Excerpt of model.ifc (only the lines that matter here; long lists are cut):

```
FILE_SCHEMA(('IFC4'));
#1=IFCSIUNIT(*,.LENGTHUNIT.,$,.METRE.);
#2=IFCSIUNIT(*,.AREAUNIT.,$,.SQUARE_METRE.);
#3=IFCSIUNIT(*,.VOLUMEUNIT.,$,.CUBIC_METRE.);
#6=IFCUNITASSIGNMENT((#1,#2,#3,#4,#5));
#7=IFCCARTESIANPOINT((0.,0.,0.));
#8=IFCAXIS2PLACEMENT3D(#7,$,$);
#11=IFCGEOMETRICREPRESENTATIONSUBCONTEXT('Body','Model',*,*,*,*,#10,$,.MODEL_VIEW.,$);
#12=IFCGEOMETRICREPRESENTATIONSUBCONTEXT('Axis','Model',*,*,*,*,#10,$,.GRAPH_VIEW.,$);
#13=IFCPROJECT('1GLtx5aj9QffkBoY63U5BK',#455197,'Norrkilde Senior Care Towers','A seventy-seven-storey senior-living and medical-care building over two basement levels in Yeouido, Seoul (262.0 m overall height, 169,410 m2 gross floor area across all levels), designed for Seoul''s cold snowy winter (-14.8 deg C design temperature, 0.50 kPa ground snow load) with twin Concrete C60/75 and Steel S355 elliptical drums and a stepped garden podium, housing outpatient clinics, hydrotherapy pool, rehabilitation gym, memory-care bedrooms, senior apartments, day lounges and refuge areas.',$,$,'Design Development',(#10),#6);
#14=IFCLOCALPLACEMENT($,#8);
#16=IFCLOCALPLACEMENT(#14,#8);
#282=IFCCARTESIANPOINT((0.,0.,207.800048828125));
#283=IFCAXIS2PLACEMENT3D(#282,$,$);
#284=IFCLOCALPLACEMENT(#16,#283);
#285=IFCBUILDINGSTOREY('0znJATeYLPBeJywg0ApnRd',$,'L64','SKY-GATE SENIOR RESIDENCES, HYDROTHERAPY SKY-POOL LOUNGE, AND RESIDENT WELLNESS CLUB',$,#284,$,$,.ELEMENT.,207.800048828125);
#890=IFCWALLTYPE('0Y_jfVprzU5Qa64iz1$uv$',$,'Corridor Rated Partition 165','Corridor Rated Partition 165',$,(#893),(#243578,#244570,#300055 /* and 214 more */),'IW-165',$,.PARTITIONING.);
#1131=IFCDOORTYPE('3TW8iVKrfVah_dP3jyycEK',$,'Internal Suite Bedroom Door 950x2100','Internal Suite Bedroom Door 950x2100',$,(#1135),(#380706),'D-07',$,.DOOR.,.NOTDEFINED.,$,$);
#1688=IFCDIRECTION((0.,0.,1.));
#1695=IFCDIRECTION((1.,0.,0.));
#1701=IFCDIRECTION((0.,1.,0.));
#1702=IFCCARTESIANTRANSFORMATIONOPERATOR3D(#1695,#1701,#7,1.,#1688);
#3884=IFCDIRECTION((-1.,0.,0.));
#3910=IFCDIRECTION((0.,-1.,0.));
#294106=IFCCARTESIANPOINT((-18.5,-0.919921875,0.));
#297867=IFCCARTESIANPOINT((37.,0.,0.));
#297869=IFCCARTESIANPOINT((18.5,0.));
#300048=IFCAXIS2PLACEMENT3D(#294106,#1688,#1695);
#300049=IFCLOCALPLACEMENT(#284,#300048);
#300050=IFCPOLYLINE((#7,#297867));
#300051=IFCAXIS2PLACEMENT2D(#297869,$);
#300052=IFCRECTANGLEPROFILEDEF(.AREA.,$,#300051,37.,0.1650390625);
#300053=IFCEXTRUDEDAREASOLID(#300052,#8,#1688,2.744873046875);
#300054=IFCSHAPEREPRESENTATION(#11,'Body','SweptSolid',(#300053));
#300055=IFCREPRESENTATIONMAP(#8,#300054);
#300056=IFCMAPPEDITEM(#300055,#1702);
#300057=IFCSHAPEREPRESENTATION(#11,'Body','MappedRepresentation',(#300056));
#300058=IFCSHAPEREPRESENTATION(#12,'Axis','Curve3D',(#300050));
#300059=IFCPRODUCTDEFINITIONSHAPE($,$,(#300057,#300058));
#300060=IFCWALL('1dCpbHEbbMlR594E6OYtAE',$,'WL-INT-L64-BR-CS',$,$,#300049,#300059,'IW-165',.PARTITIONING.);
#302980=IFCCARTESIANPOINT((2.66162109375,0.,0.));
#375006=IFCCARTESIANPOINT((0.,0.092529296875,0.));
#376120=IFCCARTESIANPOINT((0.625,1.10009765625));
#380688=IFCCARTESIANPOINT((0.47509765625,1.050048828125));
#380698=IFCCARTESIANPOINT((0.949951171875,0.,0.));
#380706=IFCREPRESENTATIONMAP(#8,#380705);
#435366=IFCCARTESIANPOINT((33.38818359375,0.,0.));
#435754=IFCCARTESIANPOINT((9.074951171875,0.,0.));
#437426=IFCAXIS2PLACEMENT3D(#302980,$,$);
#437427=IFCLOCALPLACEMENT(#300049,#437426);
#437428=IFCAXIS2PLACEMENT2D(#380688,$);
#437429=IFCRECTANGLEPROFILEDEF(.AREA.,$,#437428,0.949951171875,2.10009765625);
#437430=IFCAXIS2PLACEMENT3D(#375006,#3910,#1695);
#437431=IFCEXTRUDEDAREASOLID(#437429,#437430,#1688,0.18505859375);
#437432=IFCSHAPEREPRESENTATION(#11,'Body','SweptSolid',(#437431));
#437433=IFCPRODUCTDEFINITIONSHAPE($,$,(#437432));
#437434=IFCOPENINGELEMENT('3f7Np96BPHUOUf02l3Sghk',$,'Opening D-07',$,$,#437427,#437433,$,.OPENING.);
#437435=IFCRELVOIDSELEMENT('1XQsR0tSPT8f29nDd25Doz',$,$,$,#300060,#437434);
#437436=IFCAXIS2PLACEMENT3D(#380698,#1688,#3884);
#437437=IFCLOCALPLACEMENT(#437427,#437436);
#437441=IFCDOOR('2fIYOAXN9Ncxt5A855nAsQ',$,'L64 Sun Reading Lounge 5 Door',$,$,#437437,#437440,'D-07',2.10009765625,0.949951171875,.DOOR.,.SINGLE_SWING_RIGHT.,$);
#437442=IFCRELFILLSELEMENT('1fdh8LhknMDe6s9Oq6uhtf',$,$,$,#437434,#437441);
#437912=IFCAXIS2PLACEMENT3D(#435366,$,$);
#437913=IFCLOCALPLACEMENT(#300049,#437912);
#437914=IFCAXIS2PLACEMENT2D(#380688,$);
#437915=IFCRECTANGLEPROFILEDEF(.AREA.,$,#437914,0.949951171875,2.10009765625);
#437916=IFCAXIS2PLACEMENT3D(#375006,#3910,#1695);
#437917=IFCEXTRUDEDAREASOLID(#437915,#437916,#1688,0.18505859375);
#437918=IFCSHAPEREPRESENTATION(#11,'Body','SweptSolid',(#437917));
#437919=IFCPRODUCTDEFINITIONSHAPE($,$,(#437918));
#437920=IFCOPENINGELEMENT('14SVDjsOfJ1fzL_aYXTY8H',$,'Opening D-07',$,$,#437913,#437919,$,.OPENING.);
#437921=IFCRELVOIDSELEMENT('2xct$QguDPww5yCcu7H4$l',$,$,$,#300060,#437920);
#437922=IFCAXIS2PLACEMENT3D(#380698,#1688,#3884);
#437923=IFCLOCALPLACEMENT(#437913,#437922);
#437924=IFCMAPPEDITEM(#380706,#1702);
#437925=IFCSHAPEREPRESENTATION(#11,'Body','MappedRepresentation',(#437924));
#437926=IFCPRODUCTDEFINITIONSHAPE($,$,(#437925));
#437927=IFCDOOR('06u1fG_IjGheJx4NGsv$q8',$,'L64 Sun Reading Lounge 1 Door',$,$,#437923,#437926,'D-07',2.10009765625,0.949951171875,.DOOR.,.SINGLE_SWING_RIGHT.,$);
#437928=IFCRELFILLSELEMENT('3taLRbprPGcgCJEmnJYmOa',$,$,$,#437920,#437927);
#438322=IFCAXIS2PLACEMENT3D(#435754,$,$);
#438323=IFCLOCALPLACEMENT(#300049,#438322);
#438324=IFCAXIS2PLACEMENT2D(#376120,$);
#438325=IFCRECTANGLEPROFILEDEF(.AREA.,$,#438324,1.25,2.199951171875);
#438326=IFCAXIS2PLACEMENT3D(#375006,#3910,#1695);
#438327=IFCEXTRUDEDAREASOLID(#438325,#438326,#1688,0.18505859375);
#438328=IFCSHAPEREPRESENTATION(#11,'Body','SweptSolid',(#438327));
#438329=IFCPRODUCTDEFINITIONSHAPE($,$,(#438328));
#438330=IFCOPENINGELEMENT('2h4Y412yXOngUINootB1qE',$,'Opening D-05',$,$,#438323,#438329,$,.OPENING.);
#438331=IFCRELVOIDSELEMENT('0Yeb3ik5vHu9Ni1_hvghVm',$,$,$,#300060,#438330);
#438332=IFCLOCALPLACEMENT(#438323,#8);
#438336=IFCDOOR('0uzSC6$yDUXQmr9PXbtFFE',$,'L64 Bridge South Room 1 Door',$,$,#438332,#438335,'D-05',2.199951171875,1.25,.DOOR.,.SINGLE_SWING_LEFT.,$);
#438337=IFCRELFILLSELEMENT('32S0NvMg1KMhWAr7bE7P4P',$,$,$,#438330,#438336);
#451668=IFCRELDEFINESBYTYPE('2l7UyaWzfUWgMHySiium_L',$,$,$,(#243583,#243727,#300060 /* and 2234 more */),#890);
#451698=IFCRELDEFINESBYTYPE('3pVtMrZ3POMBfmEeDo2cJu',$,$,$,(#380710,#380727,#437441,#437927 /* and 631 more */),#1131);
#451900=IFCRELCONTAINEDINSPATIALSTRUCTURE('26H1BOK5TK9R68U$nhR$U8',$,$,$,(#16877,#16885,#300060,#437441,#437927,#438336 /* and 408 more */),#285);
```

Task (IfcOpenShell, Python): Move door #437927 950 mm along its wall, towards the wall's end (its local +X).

```python
import ifcopenshell
import ifcopenshell.api.geometry
import ifcopenshell.util.placement
import ifcopenshell.util.unit

model = ifcopenshell.open("model.ifc")
unit_scale = ifcopenshell.util.unit.calculate_unit_scale(model)

door = model.by_guid("06u1fG_IjGheJx4NGsv$q8")
opening = door.FillsVoids[0].RelatingOpeningElement
wall = opening.VoidsElements[0].RelatingBuildingElement

wall_matrix = ifcopenshell.util.placement.get_local_placement(wall.ObjectPlacement)
shift = wall_matrix[:3, 0] * 0.95 / unit_scale
before = ifcopenshell.util.placement.get_local_placement(door.ObjectPlacement)[:3, 3].copy()

# The door is placed relative to its opening, so it follows when the opening moves.
matrix = ifcopenshell.util.placement.get_local_placement(opening.ObjectPlacement)
matrix[:3, 3] += shift
ifcopenshell.api.geometry.edit_object_placement(
    model, product=opening, matrix=matrix, is_si=False, should_transform_children=True
)

after = ifcopenshell.util.placement.get_local_placement(door.ObjectPlacement)[:3, 3]
print("door moved by", (after - before).round(3) + 0.0)

model.write("model_edited.ifc")
```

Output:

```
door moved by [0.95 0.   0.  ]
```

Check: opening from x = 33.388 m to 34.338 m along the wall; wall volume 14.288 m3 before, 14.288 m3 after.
